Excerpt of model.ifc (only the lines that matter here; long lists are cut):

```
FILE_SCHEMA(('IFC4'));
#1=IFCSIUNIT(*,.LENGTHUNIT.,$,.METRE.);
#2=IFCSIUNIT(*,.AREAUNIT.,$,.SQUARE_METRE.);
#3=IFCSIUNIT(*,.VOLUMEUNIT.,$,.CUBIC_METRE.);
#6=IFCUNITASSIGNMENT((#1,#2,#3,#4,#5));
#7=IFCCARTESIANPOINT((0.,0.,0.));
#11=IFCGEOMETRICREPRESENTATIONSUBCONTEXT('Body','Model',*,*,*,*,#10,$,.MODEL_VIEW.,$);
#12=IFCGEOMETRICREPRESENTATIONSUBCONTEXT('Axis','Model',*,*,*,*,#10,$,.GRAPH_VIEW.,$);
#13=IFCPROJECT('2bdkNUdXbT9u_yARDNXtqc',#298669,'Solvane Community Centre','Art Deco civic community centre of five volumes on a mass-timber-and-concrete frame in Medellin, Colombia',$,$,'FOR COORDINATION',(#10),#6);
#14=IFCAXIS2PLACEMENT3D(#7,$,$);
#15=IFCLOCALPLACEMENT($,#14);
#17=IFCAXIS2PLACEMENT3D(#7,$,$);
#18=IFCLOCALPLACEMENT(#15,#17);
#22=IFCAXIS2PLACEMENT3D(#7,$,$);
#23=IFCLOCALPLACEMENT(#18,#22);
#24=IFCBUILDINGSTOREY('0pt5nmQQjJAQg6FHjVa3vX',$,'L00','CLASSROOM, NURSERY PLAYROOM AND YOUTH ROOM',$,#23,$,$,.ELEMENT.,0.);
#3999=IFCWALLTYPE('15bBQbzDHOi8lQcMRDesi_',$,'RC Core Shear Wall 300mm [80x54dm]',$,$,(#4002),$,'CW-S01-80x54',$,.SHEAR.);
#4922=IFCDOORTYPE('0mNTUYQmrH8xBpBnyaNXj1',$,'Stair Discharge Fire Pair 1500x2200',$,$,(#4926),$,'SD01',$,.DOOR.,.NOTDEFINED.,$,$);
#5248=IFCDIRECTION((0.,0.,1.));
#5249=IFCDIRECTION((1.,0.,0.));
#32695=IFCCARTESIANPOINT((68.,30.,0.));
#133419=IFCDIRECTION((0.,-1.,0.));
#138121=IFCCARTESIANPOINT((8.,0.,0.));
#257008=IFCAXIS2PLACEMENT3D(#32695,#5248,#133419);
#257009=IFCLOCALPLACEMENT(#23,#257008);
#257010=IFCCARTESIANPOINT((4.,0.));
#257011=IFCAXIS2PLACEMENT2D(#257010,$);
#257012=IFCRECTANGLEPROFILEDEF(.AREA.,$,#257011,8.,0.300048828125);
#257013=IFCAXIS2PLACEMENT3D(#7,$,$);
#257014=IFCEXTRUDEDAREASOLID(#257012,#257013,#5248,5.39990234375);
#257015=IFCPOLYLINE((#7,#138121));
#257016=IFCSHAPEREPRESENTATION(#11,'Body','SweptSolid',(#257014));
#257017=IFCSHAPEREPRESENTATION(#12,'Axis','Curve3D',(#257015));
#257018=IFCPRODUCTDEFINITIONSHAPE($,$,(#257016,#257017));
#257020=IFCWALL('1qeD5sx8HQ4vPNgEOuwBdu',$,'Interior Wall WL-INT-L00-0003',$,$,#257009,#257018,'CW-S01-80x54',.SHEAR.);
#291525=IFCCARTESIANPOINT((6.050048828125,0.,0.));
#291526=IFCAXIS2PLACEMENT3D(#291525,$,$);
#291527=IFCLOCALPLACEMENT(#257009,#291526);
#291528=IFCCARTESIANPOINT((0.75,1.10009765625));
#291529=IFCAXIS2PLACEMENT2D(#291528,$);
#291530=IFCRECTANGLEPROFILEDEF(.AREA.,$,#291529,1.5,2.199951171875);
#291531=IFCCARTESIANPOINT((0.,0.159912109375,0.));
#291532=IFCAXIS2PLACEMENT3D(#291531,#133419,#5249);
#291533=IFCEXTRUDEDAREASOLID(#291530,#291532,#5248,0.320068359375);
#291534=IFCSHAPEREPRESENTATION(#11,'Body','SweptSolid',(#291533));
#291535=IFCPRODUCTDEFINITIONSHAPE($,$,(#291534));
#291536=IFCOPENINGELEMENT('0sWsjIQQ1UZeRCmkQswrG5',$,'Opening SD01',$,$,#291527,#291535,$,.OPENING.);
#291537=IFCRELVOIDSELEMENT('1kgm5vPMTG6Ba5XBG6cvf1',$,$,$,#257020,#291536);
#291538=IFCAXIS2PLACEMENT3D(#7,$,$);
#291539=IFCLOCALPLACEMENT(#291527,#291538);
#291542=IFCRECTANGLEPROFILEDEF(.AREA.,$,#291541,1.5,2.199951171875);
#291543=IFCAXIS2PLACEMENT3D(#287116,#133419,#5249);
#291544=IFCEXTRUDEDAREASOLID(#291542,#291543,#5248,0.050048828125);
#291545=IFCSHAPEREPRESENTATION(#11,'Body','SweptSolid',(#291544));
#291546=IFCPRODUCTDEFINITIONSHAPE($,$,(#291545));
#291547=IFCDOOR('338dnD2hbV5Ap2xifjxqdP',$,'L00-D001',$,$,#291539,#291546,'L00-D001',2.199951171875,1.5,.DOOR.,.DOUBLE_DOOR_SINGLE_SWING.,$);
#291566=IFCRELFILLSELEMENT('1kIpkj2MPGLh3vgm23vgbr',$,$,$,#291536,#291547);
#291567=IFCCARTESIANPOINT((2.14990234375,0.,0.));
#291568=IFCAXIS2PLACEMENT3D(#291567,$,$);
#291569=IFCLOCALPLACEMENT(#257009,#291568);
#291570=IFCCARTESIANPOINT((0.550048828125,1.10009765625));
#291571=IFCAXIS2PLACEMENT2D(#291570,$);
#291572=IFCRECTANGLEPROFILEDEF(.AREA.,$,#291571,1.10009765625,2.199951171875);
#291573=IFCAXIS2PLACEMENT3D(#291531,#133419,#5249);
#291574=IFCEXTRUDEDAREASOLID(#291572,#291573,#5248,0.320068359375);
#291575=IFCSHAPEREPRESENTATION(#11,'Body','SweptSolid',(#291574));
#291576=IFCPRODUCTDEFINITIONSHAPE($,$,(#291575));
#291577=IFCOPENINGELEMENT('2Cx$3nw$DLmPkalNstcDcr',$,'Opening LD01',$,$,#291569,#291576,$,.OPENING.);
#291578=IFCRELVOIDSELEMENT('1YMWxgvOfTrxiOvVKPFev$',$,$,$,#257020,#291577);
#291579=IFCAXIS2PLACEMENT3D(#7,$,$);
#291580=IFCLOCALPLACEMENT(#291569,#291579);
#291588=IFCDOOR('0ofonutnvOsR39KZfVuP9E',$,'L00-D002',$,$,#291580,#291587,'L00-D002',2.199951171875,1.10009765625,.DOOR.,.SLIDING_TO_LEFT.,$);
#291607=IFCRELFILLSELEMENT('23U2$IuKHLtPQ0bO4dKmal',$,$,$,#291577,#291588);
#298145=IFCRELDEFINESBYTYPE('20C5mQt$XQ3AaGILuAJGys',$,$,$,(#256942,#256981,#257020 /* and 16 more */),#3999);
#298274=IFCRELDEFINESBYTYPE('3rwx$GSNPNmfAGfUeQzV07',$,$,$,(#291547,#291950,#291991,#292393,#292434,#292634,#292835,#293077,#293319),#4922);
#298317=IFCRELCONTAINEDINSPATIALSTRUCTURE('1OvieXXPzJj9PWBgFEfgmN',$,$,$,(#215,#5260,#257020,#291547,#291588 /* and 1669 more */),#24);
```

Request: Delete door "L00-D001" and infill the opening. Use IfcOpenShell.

```python
import ifcopenshell
import ifcopenshell.api.feature
import ifcopenshell.api.root
import ifcopenshell.geom
import ifcopenshell.util.shape

model = ifcopenshell.open("model.ifc")
settings = ifcopenshell.geom.settings()


def volume(element):
    """Net volume in cubic metres, openings subtracted."""
    shape = ifcopenshell.geom.create_shape(settings, element)
    return ifcopenshell.util.shape.get_volume(shape.geometry)


door = model.by_guid("338dnD2hbV5Ap2xifjxqdP")
opening = door.FillsVoids[0].RelatingOpeningElement
wall = opening.VoidsElements[0].RelatingBuildingElement
before = volume(wall)

ifcopenshell.api.root.remove_product(model, product=door)
ifcopenshell.api.feature.remove_feature(model, feature=opening)

after = volume(wall)

print(f"wall volume {before:.3f} -> {after:.3f} m3")

model.write("model-out.ifc")
```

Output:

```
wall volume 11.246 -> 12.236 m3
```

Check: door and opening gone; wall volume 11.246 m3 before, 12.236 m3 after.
